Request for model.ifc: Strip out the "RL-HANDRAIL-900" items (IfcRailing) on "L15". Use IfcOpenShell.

First a look at what the model holds.

```python
import ifcopenshell
import ifcopenshell.util.element

model = ifcopenshell.open("model.ifc")
print(model.schema)
storey = next(s for s in model.by_type("IfcBuildingStorey") if s.Name == "L15")
railings = [e for e in ifcopenshell.util.element.get_decomposition(storey) if e.is_a("IfcRailing")]
seen = {}
for e in railings:
    element_type = ifcopenshell.util.element.get_type(e)
    name = element_type.Name if element_type not in (None, e) else None
    seen[name] = seen.get(name, 0) + 1
for name, count in sorted(seen.items(), key=str):
    print(count, "x", name)
```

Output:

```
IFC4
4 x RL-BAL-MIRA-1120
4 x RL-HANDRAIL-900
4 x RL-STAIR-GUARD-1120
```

```python
import ifcopenshell
import ifcopenshell.api.root
import ifcopenshell.util.element

model = ifcopenshell.open("model.ifc")

storey = next(s for s in model.by_type("IfcBuildingStorey") if s.Name == "L15")
railings = [e for e in ifcopenshell.util.element.get_decomposition(storey) if e.is_a("IfcRailing")]
targets = [e for e in railings if (t := ifcopenshell.util.element.get_type(e)) not in (None, e) and t.Name == "RL-HANDRAIL-900"]

for e in targets:
    ifcopenshell.api.root.remove_product(model, product=e)
print(len(targets), "removed")

model.write("model_rev.ifc")
```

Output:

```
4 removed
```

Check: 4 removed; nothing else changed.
